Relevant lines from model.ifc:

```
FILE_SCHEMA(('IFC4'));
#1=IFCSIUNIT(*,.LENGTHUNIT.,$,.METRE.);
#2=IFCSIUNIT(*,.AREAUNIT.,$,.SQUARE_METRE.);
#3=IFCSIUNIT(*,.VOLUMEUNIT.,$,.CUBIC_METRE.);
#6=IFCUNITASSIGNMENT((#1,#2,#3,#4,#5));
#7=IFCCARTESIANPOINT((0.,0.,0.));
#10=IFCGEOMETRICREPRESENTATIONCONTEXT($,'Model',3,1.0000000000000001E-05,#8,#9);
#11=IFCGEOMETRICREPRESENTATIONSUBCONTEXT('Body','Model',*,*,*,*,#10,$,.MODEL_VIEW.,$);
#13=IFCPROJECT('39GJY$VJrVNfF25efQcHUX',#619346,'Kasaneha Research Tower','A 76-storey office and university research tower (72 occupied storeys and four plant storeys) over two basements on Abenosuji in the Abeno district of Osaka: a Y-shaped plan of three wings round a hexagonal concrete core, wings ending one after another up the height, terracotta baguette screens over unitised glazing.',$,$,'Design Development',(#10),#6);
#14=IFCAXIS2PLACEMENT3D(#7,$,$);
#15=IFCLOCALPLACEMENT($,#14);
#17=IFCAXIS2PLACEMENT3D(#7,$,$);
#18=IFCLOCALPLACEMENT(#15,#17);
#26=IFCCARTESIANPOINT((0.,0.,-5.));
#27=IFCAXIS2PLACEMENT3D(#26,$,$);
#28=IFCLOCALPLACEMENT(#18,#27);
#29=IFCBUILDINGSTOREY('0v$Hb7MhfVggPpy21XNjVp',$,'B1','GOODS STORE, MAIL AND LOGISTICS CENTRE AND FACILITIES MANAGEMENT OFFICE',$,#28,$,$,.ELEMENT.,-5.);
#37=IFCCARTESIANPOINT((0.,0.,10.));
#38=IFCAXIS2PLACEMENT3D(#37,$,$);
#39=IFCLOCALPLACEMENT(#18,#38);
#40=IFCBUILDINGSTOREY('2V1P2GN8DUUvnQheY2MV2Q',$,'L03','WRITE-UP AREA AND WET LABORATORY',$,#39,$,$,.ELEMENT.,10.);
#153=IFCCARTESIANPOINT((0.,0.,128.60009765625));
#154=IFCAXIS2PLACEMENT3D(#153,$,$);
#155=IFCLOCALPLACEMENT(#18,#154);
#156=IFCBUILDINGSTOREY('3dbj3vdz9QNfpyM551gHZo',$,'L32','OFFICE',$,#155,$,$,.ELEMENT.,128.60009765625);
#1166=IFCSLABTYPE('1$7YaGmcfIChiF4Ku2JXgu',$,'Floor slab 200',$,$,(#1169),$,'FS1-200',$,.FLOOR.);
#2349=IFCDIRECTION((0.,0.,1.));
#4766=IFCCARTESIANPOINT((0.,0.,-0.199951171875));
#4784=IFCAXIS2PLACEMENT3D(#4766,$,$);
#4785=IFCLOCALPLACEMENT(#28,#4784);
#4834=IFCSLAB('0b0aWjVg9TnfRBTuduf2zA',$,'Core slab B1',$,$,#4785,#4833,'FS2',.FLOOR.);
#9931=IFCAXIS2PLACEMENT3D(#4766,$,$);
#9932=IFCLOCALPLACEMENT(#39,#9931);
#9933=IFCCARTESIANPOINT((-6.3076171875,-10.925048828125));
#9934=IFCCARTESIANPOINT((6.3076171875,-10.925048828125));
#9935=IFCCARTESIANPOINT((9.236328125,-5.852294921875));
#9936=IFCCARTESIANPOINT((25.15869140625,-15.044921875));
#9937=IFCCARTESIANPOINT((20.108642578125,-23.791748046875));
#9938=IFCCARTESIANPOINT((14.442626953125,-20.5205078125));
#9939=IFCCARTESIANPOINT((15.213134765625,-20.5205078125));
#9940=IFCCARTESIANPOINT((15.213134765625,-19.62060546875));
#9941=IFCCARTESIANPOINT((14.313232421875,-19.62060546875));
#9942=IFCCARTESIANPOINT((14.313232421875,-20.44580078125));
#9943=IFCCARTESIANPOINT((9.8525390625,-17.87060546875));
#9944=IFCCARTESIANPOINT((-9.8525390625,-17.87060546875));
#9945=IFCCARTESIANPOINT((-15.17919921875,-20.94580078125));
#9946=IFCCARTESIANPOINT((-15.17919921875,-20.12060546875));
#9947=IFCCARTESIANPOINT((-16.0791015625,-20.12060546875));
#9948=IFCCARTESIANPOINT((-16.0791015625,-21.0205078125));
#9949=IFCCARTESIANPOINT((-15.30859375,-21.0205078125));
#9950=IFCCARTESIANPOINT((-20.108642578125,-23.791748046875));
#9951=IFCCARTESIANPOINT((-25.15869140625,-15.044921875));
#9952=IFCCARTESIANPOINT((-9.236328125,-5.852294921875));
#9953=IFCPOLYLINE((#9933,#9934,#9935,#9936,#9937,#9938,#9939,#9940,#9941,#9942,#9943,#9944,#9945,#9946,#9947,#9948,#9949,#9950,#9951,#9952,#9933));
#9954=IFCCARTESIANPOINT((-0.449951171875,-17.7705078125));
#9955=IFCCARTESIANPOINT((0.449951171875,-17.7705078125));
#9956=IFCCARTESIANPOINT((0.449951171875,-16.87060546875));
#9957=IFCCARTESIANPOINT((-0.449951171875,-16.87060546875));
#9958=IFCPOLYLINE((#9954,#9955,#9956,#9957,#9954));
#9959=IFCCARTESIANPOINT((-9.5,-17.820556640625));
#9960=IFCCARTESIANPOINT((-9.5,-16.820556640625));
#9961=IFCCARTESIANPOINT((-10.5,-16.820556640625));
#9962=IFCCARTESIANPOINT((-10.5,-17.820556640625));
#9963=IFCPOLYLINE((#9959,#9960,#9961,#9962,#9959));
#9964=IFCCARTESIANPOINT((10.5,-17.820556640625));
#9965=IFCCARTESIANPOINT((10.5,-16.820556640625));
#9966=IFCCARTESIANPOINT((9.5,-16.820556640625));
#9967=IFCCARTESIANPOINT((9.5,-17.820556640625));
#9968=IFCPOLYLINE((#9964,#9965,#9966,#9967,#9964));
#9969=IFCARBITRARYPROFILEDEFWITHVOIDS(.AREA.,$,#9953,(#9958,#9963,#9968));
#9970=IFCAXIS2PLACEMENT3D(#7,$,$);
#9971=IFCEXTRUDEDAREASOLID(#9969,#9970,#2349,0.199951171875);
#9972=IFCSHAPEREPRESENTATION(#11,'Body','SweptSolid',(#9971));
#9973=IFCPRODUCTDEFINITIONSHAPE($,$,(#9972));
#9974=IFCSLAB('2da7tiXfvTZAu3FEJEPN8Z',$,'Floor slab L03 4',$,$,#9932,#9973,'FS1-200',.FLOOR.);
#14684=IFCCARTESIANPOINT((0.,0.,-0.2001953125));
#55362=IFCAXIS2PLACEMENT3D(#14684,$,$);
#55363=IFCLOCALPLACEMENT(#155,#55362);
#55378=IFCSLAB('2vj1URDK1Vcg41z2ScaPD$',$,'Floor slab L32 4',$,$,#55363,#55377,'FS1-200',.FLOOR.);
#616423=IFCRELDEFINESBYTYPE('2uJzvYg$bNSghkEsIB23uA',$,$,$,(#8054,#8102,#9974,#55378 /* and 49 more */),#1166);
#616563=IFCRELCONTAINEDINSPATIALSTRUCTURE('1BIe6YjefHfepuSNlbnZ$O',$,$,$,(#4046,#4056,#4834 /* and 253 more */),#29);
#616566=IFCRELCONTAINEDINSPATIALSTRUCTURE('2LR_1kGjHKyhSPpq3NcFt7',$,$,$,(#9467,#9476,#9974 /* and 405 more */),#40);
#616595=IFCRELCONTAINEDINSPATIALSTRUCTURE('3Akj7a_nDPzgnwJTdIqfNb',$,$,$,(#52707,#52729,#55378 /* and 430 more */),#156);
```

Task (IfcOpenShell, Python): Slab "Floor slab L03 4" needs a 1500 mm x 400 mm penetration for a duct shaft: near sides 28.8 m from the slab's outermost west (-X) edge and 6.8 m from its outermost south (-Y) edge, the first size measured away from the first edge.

```python
import numpy as np
import ifcopenshell
import ifcopenshell.api.feature
import ifcopenshell.api.geometry
import ifcopenshell.api.root
import ifcopenshell.geom
import ifcopenshell.util.placement
import ifcopenshell.util.representation
import ifcopenshell.util.shape
import ifcopenshell.util.unit

model = ifcopenshell.open("model.ifc")
unit_scale = ifcopenshell.util.unit.calculate_unit_scale(model)
settings = ifcopenshell.geom.settings()


def volume(element):
    """Net volume in cubic metres, openings subtracted."""
    shape = ifcopenshell.geom.create_shape(settings, element)
    return ifcopenshell.util.shape.get_volume(shape.geometry)


slab = model.by_guid("2da7tiXfvTZAu3FEJEPN8Z")
before = volume(slab)

# Extent in the slab's own axes, in metres. The edges named are its -X and -Y sides.
slab_shape = ifcopenshell.geom.create_shape(settings, slab)
vertices = ifcopenshell.util.shape.get_vertices(slab_shape.geometry)
x_min, y_min, bottom = vertices.min(axis=0)
top = vertices[:, 2].max()

opening = ifcopenshell.api.root.create_entity(model, ifc_class="IfcOpeningElement", name="Duct shaft opening", predefined_type="OPENING")
context = ifcopenshell.util.representation.get_context(model, "Model", "Body", "MODEL_VIEW")
width, depth = 1.5, 0.4
outline = [(0.0, 0.0), (width, 0.0), (width, depth), (0.0, depth), (0.0, 0.0)]
# Overshoot both faces by 50 mm so the cut is clean.
shape = ifcopenshell.api.geometry.add_slab_representation(
    model, context=context, depth=top - bottom + 0.1, polyline=outline
)
ifcopenshell.api.geometry.assign_representation(model, product=opening, representation=shape)

matrix = ifcopenshell.util.placement.get_local_placement(slab.ObjectPlacement)
matrix[:, 3] = matrix @ np.append(np.array([x_min + 28.8, y_min + 6.8, bottom - 0.05]) / unit_scale, 1.0)
ifcopenshell.api.geometry.edit_object_placement(model, product=opening, matrix=matrix, is_si=False)
ifcopenshell.api.feature.add_feature(model, feature=opening, element=slab)

after = volume(slab)

print(f"slab volume {before:.3f} -> {after:.3f} m3")

model.write("model_updated.ifc")
```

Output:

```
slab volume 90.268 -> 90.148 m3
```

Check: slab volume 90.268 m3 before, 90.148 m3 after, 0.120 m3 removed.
